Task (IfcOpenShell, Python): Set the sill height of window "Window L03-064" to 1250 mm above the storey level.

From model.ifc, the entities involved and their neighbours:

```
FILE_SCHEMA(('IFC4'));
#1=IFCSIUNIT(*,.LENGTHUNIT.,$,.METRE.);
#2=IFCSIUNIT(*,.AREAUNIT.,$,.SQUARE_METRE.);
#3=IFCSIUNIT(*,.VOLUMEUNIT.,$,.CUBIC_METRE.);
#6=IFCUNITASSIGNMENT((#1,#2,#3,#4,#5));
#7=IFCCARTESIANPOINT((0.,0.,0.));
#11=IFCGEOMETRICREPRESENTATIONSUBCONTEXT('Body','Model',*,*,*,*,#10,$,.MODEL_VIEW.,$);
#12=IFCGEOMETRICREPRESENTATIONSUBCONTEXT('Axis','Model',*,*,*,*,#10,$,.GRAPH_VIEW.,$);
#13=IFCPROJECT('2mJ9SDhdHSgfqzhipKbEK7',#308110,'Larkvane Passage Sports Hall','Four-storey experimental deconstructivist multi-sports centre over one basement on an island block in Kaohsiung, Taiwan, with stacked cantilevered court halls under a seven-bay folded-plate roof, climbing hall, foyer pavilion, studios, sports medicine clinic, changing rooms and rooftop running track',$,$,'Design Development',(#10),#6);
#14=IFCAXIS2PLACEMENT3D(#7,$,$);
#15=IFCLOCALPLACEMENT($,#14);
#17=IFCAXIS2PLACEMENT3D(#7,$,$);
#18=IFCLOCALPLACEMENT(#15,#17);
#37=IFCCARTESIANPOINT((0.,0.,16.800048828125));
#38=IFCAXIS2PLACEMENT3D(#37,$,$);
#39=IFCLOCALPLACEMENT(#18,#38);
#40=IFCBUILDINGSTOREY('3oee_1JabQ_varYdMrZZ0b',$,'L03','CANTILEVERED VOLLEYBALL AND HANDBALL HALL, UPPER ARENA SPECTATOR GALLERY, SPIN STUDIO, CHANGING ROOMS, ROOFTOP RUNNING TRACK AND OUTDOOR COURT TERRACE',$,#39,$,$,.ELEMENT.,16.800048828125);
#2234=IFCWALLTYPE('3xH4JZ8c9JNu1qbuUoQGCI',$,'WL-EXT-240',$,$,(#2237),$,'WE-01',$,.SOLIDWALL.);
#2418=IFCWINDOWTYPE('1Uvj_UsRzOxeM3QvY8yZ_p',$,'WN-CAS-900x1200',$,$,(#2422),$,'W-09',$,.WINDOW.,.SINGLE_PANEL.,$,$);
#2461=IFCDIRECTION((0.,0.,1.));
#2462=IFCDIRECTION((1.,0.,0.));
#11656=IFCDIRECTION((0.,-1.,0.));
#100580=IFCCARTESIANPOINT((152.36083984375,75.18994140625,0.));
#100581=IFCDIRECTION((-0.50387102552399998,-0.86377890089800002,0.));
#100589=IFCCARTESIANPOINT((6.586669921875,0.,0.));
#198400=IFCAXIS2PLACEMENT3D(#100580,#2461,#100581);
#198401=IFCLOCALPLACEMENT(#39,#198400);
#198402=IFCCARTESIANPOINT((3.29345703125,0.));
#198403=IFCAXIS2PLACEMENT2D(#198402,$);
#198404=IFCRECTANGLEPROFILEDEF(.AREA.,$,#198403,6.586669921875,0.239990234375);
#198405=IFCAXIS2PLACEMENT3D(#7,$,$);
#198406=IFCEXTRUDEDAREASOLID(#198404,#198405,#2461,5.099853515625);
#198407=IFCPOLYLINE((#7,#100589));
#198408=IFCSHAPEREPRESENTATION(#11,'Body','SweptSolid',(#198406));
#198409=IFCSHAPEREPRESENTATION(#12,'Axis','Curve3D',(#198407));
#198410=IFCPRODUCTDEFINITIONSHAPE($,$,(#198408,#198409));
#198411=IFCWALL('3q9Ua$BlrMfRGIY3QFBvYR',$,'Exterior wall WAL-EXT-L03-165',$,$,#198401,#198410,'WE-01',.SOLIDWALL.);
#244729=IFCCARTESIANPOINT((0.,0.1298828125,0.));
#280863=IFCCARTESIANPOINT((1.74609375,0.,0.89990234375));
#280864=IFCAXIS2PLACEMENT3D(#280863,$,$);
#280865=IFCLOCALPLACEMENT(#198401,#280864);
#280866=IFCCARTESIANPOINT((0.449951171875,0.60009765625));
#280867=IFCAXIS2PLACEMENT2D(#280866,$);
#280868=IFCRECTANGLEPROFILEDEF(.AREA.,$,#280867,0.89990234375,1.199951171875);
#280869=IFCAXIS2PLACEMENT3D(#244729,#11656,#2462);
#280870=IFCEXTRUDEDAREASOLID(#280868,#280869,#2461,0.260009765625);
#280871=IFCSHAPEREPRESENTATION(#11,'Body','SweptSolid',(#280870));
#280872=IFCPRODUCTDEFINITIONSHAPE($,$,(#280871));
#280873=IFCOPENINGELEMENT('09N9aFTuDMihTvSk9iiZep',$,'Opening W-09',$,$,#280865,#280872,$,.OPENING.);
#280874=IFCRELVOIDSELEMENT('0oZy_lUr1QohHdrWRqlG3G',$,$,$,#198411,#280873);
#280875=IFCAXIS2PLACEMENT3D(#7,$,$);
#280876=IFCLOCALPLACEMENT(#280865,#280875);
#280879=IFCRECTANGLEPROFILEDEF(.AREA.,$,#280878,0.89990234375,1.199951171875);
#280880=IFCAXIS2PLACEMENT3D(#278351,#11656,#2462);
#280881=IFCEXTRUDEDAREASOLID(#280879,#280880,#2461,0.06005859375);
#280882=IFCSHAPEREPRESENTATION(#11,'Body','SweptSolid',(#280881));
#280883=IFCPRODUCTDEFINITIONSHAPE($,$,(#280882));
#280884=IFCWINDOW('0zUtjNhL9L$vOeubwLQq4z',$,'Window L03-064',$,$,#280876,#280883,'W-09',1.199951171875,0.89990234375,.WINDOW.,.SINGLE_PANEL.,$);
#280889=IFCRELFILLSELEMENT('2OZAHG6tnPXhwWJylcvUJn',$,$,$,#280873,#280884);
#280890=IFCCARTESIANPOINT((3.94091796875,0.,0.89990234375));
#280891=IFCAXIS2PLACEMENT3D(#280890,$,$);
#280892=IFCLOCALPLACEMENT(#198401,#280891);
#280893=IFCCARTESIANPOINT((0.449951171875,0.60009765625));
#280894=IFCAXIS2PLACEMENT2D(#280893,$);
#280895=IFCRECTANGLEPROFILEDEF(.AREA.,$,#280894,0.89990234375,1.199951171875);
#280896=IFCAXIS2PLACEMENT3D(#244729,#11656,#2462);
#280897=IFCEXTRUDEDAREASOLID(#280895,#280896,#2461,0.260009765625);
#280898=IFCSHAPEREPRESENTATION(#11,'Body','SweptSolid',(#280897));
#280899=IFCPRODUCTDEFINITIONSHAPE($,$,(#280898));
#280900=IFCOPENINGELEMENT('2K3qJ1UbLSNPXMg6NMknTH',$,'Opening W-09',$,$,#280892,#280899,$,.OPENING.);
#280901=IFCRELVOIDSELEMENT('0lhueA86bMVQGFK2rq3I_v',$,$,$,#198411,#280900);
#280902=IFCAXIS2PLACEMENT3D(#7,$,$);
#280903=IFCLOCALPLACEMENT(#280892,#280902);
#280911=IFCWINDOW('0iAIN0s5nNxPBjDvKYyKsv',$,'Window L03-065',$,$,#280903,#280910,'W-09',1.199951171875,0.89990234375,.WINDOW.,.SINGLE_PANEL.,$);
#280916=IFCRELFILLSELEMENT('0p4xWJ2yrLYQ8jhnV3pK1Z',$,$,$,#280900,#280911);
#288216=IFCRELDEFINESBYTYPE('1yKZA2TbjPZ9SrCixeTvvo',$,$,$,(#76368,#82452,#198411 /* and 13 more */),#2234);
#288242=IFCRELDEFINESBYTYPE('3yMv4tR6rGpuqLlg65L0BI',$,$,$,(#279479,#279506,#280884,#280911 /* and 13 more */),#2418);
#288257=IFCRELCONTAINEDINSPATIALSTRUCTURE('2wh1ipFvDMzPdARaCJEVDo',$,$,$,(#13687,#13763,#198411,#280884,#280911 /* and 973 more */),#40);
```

```python
import numpy as np
import ifcopenshell
import ifcopenshell.api.geometry
import ifcopenshell.geom
import ifcopenshell.util.element
import ifcopenshell.util.placement
import ifcopenshell.util.shape
import ifcopenshell.util.unit

model = ifcopenshell.open("model.ifc")
unit_scale = ifcopenshell.util.unit.calculate_unit_scale(model)

window = model.by_guid("0zUtjNhL9L$vOeubwLQq4z")
opening = window.FillsVoids[0].RelatingOpeningElement
storey = ifcopenshell.util.element.get_container(window, ifc_class="IfcBuildingStorey")
level = ifcopenshell.util.placement.get_local_placement(storey.ObjectPlacement)[2, 3]

# The opening's origin need not be at the sill, so measure its lowest point.
shape = ifcopenshell.geom.create_shape(ifcopenshell.geom.settings(), opening)
bottom = ifcopenshell.util.shape.get_shape_bottom_elevation(shape, shape.geometry) / unit_scale
dz = level + 1.25 - bottom

shift = np.array([0.0, 0.0, dz])
# The window is placed relative to its opening, so it follows when the opening moves.
matrix = ifcopenshell.util.placement.get_local_placement(opening.ObjectPlacement)
matrix[:3, 3] += shift
ifcopenshell.api.geometry.edit_object_placement(
    model, product=opening, matrix=matrix, is_si=False, should_transform_children=True
)

print(f"moved by {dz * unit_scale:+.3f} m")

model.write("model_updated.ifc")
```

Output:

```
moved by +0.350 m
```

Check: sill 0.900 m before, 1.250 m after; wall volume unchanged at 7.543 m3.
